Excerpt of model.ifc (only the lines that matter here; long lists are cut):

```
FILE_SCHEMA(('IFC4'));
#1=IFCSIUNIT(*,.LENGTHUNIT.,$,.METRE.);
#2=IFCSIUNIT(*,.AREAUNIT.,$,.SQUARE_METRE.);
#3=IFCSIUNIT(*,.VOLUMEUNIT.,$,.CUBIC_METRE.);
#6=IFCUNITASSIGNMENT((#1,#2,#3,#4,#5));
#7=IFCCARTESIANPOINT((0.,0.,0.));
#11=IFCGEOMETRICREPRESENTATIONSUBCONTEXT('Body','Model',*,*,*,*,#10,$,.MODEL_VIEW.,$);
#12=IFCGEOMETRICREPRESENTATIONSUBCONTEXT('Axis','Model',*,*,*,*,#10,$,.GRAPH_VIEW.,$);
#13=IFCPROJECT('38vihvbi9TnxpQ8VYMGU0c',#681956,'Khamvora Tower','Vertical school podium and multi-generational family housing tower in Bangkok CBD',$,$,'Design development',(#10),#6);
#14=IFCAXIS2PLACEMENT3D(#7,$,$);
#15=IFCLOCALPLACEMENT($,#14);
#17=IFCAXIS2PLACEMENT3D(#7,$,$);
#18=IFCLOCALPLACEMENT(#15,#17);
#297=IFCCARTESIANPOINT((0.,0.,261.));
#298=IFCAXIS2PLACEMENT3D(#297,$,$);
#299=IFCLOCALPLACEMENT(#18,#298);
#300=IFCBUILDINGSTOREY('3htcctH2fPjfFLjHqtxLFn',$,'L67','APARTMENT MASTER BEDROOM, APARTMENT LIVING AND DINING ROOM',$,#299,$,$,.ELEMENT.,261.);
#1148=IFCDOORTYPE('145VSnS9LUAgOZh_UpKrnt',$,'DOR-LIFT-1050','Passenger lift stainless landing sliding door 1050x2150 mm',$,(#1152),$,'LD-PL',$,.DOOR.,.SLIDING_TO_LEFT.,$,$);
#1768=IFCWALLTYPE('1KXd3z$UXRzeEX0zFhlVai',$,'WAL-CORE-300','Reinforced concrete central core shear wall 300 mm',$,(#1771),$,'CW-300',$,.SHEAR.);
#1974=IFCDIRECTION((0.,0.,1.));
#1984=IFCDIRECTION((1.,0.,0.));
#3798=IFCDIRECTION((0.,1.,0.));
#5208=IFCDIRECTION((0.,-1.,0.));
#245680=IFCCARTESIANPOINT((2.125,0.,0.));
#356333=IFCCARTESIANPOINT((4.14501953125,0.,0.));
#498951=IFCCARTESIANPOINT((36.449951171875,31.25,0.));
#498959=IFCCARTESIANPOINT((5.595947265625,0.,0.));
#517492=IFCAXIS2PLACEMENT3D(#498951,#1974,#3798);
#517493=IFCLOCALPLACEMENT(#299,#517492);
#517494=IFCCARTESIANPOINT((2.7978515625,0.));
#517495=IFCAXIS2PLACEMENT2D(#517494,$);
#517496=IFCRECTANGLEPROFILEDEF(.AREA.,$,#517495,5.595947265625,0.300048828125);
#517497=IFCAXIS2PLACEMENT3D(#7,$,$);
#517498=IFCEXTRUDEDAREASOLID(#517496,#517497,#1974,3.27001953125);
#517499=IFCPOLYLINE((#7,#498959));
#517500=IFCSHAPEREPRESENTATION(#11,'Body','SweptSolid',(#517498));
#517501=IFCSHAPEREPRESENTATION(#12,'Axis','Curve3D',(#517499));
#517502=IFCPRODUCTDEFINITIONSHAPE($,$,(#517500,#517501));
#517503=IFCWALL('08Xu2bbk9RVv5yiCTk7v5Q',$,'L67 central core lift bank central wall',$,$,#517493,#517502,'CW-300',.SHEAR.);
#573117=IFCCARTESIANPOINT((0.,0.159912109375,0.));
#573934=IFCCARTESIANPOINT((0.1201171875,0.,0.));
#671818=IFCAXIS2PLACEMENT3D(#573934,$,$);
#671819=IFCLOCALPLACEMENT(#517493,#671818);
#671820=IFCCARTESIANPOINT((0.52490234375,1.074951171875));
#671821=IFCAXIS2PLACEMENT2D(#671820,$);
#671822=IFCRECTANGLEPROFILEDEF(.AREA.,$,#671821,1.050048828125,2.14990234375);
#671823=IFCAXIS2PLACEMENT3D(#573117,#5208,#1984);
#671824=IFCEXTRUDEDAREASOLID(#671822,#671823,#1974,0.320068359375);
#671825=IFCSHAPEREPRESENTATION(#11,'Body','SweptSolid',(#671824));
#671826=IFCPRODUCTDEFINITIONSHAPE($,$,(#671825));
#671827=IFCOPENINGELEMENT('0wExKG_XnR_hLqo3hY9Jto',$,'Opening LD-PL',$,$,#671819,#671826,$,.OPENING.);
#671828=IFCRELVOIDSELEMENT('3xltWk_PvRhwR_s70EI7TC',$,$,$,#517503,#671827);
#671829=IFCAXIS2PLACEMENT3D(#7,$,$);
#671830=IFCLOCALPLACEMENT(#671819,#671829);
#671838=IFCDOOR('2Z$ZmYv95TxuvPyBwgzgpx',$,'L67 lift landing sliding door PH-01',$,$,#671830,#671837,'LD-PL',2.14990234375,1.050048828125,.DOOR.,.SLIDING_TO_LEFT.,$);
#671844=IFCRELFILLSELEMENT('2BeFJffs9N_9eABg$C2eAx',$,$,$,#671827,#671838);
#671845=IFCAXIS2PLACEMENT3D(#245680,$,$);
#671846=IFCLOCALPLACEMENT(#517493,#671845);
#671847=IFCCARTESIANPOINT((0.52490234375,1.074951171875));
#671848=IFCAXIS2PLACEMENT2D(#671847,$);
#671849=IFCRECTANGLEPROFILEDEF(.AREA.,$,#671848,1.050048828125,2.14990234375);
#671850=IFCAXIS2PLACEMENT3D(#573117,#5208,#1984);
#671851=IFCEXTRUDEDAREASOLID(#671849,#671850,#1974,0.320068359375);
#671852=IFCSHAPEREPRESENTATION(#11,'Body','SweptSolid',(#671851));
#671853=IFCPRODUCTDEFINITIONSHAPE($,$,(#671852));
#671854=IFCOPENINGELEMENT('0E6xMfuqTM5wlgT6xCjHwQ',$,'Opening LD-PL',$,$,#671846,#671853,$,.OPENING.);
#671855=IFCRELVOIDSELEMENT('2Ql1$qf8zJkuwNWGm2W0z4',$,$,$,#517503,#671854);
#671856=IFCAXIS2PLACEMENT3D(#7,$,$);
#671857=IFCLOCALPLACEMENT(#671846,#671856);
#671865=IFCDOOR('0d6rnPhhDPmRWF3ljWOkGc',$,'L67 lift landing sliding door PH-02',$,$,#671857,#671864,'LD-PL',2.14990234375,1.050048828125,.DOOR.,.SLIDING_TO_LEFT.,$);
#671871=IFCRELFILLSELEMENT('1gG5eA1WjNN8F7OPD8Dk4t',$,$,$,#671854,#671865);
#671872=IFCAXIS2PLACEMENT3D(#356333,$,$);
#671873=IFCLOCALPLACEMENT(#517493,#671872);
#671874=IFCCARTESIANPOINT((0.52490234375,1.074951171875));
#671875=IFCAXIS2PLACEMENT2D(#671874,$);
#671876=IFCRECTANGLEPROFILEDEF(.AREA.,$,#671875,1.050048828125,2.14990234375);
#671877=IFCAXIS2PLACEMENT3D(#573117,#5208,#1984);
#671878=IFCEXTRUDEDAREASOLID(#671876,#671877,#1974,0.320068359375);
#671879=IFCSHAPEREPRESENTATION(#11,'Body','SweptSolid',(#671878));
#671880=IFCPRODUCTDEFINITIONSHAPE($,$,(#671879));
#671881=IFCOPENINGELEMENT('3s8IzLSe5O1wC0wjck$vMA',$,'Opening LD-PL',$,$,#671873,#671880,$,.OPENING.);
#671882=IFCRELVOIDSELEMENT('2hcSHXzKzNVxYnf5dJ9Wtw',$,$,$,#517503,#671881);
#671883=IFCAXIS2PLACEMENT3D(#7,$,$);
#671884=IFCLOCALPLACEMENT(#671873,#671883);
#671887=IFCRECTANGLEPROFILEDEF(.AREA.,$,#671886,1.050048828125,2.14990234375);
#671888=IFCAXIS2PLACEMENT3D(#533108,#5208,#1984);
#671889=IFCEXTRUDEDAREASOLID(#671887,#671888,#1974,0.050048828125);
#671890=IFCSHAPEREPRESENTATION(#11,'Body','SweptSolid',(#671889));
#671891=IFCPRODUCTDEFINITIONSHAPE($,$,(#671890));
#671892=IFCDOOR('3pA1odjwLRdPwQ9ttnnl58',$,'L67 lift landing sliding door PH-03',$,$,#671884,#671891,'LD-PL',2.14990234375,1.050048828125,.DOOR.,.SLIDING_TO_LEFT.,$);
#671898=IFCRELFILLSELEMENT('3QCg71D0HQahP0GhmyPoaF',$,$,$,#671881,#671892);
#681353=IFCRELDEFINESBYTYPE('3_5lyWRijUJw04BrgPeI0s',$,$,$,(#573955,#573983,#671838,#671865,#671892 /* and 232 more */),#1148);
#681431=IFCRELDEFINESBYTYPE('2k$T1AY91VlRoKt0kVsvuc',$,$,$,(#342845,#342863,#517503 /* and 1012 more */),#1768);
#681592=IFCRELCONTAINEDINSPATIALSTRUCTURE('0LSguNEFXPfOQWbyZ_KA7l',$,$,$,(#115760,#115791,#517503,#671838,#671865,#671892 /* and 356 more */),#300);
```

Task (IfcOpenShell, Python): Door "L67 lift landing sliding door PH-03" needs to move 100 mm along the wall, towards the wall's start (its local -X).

```python
import ifcopenshell
import ifcopenshell.api.geometry
import ifcopenshell.util.placement

model = ifcopenshell.open("model.ifc")

door = model.by_guid("3pA1odjwLRdPwQ9ttnnl58")
opening = door.FillsVoids[0].RelatingOpeningElement
wall = opening.VoidsElements[0].RelatingBuildingElement

wall_matrix = ifcopenshell.util.placement.get_local_placement(wall.ObjectPlacement)
shift = wall_matrix[:3, 0] * -0.1
before = ifcopenshell.util.placement.get_local_placement(door.ObjectPlacement)[:3, 3].copy()

# The door is placed relative to its opening, so it follows when the opening moves.
matrix = ifcopenshell.util.placement.get_local_placement(opening.ObjectPlacement)
matrix[:3, 3] += shift
ifcopenshell.api.geometry.edit_object_placement(
    model, product=opening, matrix=matrix, is_si=False, should_transform_children=True
)

after = ifcopenshell.util.placement.get_local_placement(door.ObjectPlacement)[:3, 3]
print("door moved by", (after - before).round(3) + 0.0)

model.write("model_rev.ifc")
```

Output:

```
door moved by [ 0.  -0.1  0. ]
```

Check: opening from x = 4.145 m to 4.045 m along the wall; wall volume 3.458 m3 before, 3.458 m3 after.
